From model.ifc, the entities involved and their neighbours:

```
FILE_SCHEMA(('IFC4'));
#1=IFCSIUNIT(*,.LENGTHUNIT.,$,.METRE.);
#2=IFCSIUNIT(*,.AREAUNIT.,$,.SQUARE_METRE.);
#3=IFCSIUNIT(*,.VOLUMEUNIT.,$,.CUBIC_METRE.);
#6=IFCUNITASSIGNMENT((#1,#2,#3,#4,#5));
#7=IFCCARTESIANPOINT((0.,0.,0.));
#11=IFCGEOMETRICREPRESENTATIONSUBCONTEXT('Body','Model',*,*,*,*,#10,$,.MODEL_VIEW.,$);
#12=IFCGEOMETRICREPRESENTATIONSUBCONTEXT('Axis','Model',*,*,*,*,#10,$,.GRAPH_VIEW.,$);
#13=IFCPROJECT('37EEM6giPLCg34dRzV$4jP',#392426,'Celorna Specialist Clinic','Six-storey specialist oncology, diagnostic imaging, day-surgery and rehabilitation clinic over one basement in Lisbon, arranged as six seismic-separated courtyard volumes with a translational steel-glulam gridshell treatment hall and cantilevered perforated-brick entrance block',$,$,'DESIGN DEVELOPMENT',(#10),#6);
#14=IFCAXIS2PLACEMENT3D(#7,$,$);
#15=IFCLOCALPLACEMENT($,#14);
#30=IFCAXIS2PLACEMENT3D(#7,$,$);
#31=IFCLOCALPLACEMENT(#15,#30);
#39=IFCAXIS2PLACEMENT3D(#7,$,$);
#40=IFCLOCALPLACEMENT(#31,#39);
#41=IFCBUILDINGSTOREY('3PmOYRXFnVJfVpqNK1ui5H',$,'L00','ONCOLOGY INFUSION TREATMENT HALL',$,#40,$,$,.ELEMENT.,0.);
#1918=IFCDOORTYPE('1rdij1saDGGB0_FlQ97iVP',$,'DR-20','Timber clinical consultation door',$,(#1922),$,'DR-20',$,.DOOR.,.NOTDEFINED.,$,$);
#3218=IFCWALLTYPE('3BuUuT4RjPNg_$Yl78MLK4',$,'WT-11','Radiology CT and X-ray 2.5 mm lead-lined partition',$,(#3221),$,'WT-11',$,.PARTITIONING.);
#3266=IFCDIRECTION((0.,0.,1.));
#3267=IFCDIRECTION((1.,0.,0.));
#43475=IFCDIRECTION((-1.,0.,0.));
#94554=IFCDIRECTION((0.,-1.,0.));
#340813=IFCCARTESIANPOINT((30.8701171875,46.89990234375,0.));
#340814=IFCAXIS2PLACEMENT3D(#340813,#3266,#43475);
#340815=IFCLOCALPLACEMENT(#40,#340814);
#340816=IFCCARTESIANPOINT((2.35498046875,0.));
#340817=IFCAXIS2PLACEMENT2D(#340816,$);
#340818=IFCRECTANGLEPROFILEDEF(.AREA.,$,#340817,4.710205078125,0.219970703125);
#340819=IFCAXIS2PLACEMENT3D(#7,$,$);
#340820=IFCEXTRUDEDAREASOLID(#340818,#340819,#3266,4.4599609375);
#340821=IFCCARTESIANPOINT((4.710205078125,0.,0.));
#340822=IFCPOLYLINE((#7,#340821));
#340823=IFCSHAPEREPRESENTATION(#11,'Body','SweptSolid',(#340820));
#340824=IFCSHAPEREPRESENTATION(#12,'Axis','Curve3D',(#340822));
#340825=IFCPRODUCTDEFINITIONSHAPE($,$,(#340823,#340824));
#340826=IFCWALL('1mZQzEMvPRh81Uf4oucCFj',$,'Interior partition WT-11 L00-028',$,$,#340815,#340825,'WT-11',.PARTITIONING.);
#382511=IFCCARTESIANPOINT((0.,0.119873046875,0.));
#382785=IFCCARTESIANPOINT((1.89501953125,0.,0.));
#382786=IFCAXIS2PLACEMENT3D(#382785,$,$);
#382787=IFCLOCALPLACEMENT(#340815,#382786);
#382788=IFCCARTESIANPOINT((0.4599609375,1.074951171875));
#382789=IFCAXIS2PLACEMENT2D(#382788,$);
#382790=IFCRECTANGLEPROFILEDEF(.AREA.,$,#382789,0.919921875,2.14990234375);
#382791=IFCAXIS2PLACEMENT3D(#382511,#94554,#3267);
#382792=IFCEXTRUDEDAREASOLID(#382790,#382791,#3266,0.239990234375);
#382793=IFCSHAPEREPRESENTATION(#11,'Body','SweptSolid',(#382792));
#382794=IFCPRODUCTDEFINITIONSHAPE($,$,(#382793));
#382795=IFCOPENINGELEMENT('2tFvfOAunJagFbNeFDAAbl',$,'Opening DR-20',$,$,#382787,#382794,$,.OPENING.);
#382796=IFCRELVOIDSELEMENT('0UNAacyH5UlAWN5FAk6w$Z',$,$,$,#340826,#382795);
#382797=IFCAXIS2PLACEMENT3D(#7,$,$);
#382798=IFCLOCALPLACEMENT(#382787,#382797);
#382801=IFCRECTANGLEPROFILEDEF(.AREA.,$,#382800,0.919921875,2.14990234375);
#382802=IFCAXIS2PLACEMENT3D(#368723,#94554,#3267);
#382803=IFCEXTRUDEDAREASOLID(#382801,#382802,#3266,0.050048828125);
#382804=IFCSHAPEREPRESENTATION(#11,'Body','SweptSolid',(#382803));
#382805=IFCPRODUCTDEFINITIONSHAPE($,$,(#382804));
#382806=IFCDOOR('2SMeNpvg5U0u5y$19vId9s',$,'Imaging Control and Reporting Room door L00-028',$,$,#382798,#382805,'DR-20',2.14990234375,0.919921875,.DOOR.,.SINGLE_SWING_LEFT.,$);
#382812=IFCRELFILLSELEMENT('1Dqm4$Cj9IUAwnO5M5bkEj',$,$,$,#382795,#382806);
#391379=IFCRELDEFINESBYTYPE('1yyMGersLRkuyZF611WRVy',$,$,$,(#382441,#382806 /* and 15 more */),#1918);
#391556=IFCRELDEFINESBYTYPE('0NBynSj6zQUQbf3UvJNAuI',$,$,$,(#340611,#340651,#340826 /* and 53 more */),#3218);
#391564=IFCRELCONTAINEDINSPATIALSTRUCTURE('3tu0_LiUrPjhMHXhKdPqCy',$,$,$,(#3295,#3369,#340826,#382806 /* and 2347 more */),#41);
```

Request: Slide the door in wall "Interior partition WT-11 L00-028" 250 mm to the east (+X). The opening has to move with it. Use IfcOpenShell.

```python
import ifcopenshell
import ifcopenshell.api.geometry
import ifcopenshell.util.placement

model = ifcopenshell.open("model.ifc")

door = model.by_guid("2SMeNpvg5U0u5y$19vId9s")
opening = door.FillsVoids[0].RelatingOpeningElement
wall = opening.VoidsElements[0].RelatingBuildingElement

wall_matrix = ifcopenshell.util.placement.get_local_placement(wall.ObjectPlacement)
shift = wall_matrix[:3, 0] * -0.25
before = ifcopenshell.util.placement.get_local_placement(door.ObjectPlacement)[:3, 3].copy()

# The door is placed relative to its opening, so it follows when the opening moves.
matrix = ifcopenshell.util.placement.get_local_placement(opening.ObjectPlacement)
matrix[:3, 3] += shift
ifcopenshell.api.geometry.edit_object_placement(
    model, product=opening, matrix=matrix, is_si=False, should_transform_children=True
)

after = ifcopenshell.util.placement.get_local_placement(door.ObjectPlacement)[:3, 3]
print("door moved by", (after - before).round(3) + 0.0)

model.write("model_edited.ifc")
```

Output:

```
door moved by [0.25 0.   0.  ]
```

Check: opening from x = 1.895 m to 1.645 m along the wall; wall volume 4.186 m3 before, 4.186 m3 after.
